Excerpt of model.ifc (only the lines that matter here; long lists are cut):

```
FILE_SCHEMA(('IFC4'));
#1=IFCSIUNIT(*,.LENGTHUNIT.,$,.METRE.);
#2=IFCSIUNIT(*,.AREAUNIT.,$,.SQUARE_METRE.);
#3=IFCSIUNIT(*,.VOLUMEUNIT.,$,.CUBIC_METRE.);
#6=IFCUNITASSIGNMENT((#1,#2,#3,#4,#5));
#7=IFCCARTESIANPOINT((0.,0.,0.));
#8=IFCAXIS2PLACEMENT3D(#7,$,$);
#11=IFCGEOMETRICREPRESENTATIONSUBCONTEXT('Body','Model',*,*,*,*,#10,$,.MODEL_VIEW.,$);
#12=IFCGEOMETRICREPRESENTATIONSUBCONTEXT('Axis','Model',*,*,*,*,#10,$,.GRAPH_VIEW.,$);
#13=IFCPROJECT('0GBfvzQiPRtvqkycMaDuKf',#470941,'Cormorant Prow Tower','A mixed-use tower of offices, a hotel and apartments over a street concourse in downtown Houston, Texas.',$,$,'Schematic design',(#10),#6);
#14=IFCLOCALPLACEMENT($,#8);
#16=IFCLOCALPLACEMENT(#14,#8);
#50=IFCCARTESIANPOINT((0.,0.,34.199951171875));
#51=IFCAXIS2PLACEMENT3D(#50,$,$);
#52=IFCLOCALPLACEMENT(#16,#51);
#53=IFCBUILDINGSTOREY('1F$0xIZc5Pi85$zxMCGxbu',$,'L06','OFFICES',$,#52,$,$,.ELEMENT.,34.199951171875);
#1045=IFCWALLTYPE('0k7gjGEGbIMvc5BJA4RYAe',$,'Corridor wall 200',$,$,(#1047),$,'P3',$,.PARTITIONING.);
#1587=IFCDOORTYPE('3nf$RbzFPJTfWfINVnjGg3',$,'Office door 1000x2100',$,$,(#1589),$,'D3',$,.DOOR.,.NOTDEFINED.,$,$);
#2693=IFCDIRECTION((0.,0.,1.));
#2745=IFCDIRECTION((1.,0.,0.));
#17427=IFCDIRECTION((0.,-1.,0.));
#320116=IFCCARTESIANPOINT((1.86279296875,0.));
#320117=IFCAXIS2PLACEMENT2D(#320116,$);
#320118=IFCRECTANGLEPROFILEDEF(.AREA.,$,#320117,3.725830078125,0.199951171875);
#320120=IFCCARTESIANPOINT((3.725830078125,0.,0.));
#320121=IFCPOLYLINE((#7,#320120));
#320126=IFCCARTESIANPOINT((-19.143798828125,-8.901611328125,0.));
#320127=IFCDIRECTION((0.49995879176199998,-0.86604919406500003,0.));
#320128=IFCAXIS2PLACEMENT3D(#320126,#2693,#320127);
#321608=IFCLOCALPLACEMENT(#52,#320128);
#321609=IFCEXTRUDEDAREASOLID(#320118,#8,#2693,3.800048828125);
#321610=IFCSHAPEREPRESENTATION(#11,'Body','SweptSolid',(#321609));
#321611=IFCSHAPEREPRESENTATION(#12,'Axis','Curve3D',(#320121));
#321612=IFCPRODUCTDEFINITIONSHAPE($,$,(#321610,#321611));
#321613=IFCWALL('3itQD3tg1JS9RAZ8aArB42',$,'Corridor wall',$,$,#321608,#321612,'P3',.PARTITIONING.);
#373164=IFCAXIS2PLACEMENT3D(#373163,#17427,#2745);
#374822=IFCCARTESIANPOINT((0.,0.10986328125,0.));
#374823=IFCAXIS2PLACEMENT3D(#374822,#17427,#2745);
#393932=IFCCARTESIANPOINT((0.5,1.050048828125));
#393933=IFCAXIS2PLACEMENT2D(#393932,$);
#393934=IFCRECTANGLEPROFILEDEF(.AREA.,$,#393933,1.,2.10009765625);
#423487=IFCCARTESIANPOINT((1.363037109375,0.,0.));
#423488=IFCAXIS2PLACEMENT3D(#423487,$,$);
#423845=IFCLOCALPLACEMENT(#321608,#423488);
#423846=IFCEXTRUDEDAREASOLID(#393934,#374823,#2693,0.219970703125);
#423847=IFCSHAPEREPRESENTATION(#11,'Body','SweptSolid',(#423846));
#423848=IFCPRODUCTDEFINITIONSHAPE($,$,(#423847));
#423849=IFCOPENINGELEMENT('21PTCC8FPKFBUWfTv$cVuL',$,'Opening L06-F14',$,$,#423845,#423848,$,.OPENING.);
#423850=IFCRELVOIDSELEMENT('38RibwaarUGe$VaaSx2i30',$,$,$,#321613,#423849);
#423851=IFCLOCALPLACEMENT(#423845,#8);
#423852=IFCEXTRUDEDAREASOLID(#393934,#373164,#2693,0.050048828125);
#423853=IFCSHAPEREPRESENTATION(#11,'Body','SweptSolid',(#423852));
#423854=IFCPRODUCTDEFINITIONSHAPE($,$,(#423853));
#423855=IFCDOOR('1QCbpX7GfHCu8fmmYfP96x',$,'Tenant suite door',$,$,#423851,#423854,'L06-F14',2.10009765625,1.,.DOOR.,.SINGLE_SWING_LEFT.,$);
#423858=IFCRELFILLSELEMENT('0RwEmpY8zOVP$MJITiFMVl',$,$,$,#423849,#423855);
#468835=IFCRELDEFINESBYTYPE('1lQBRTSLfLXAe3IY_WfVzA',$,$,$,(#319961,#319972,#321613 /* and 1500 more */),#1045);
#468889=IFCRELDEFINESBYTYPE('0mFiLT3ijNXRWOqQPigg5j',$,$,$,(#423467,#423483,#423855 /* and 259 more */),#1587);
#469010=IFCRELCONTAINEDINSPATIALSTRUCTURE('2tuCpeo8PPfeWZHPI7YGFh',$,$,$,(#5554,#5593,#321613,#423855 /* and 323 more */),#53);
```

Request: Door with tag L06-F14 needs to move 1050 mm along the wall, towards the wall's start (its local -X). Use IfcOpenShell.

```python
import ifcopenshell
import ifcopenshell.api.geometry
import ifcopenshell.util.placement

model = ifcopenshell.open("model.ifc")

door = model.by_id(423855)
opening = door.FillsVoids[0].RelatingOpeningElement
wall = opening.VoidsElements[0].RelatingBuildingElement

wall_matrix = ifcopenshell.util.placement.get_local_placement(wall.ObjectPlacement)
shift = wall_matrix[:3, 0] * -1.05
before = ifcopenshell.util.placement.get_local_placement(door.ObjectPlacement)[:3, 3].copy()

# The door is placed relative to its opening, so it follows when the opening moves.
matrix = ifcopenshell.util.placement.get_local_placement(opening.ObjectPlacement)
matrix[:3, 3] += shift
ifcopenshell.api.geometry.edit_object_placement(
    model, product=opening, matrix=matrix, is_si=False, should_transform_children=True
)

after = ifcopenshell.util.placement.get_local_placement(door.ObjectPlacement)[:3, 3]
print("door moved by", (after - before).round(3) + 0.0)

model.write("model-out.ifc")
```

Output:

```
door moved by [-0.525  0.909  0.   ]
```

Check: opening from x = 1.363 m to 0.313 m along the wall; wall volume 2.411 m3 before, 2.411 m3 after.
